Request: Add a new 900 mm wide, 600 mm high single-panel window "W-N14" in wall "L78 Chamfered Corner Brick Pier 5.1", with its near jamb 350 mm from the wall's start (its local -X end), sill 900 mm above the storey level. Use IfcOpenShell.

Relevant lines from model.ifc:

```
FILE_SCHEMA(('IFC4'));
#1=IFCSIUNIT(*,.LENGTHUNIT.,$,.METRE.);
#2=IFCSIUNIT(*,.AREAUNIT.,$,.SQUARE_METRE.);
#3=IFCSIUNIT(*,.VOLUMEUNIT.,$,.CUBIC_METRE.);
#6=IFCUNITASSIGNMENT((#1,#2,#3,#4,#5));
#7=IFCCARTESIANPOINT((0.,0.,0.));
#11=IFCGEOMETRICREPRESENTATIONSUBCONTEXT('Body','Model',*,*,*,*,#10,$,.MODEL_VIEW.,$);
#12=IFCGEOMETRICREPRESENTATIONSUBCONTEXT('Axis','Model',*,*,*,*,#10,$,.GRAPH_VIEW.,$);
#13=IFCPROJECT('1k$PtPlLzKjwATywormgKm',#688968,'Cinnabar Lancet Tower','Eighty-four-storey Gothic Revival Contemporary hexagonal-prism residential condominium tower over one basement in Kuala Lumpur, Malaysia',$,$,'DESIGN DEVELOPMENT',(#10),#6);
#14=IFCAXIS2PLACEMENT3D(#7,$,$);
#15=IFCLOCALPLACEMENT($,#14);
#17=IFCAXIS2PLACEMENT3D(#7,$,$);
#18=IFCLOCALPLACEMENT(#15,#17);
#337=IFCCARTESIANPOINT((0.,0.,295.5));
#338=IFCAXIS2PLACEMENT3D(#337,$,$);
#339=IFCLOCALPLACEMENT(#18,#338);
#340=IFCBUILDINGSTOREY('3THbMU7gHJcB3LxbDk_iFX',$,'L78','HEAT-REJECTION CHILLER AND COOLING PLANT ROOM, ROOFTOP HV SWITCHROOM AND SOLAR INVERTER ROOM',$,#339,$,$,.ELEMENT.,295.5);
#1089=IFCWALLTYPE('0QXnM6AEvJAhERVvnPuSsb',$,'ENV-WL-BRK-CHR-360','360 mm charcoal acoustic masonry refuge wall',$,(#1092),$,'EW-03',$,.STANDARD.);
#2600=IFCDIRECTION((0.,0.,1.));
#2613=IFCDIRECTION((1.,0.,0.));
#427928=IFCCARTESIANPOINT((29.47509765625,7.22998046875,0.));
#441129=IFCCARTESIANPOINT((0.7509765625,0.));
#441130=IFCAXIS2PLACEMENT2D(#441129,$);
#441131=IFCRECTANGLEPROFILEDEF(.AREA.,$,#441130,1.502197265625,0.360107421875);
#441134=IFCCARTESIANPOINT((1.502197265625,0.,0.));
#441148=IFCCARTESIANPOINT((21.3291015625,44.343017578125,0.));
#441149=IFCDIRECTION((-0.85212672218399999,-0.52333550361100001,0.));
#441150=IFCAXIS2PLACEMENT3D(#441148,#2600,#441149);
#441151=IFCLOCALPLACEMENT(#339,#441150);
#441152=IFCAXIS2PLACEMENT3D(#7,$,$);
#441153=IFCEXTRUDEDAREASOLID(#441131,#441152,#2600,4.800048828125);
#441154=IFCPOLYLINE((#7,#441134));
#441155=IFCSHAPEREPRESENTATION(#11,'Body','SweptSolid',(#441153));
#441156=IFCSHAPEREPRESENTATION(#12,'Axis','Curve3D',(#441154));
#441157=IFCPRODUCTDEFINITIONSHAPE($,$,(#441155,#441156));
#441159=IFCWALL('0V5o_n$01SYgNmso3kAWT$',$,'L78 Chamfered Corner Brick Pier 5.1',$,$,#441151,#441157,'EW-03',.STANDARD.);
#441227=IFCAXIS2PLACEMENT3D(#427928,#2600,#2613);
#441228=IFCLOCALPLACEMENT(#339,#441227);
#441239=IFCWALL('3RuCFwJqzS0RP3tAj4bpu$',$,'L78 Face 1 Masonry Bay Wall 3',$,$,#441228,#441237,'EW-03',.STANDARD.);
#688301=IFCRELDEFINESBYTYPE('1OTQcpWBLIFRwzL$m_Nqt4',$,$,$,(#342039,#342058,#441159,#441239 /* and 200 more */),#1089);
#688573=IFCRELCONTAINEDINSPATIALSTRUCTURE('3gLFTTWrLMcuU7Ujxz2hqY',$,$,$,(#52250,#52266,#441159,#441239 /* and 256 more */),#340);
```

```python
import numpy as np
import ifcopenshell
import ifcopenshell.api.feature
import ifcopenshell.api.geometry
import ifcopenshell.api.root
import ifcopenshell.api.spatial
import ifcopenshell.geom
import ifcopenshell.util.element
import ifcopenshell.util.placement
import ifcopenshell.util.representation
import ifcopenshell.util.shape
import ifcopenshell.util.unit

model = ifcopenshell.open("model.ifc")
unit_scale = ifcopenshell.util.unit.calculate_unit_scale(model)
settings = ifcopenshell.geom.settings()


def volume(element):
    """Net volume in cubic metres, openings subtracted."""
    shape = ifcopenshell.geom.create_shape(settings, element)
    return ifcopenshell.util.shape.get_volume(shape.geometry)


wall = model.by_guid("0V5o_n$01SYgNmso3kAWT$")
storey = ifcopenshell.util.element.get_container(wall, ifc_class="IfcBuildingStorey")
context = ifcopenshell.util.representation.get_context(model, "Model", "Body", "MODEL_VIEW")
before = volume(wall)

width, height, from_end, sill = 0.9, 0.6, 0.35, 0.9  # metres

# The wall runs along its own X axis, and the end named is its -X end.
wall_shape = ifcopenshell.geom.create_shape(settings, wall)
x, y, z = ifcopenshell.util.shape.get_vertices(wall_shape.geometry).T
start = x.min() + from_end
face, thickness = float(y.min()), float(y.max() - y.min())
wall_matrix = ifcopenshell.util.placement.get_local_placement(wall.ObjectPlacement)
level = ifcopenshell.util.placement.get_local_placement(storey.ObjectPlacement)[2, 3]


def in_wall(x, y):
    """Placement at x, y metres in the wall's axes, at sill height."""
    matrix = wall_matrix.copy()
    matrix[:, 3] = wall_matrix @ np.array([x / unit_scale, y / unit_scale, 0.0, 1.0])
    matrix[2, 3] = level + sill / unit_scale
    return matrix


# Opening: a box that overshoots both wall faces by 50 mm.
opening = ifcopenshell.api.root.create_entity(model, ifc_class="IfcOpeningElement", predefined_type="OPENING")
box = ifcopenshell.api.geometry.add_wall_representation(
    model, context=context, length=width, height=height, thickness=thickness + 0.1
)
ifcopenshell.api.geometry.assign_representation(model, product=opening, representation=box)
ifcopenshell.api.geometry.edit_object_placement(model, product=opening, matrix=in_wall(start, face - 0.05), is_si=False)
ifcopenshell.api.feature.add_feature(model, feature=opening, element=wall)

window = ifcopenshell.api.root.create_entity(model, ifc_class="IfcWindow", name="W-N14", predefined_type="WINDOW")
window.OverallWidth, window.OverallHeight = width / unit_scale, height / unit_scale
window.PartitioningType = "SINGLE_PANEL"
body = ifcopenshell.api.geometry.add_window_representation(
    model,
    context=context,
    overall_width=window.OverallWidth,
    overall_height=window.OverallHeight,
    partition_type="SINGLE_PANEL",
)
ifcopenshell.api.geometry.assign_representation(model, product=window, representation=body)
ifcopenshell.api.spatial.assign_container(model, products=[window], relating_structure=storey)
ifcopenshell.api.feature.add_filling(model, opening=opening, element=window)

# Centre the window in the wall's thickness.
ifcopenshell.api.geometry.edit_object_placement(model, product=window, matrix=in_wall(start, face), is_si=False)
window_shape = ifcopenshell.geom.create_shape(settings, window)
depth = ifcopenshell.util.shape.get_vertices(window_shape.geometry)[:, 1]
offset = face + thickness / 2 - (depth.min() + depth.max()) / 2
ifcopenshell.api.geometry.edit_object_placement(model, product=window, matrix=in_wall(start, offset), is_si=False)

after = volume(wall)

print(f"wall volume {before:.3f} -> {after:.3f} m3")

model.write("model-out.ifc")
```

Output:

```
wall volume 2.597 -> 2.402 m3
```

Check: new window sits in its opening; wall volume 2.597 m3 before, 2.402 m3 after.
